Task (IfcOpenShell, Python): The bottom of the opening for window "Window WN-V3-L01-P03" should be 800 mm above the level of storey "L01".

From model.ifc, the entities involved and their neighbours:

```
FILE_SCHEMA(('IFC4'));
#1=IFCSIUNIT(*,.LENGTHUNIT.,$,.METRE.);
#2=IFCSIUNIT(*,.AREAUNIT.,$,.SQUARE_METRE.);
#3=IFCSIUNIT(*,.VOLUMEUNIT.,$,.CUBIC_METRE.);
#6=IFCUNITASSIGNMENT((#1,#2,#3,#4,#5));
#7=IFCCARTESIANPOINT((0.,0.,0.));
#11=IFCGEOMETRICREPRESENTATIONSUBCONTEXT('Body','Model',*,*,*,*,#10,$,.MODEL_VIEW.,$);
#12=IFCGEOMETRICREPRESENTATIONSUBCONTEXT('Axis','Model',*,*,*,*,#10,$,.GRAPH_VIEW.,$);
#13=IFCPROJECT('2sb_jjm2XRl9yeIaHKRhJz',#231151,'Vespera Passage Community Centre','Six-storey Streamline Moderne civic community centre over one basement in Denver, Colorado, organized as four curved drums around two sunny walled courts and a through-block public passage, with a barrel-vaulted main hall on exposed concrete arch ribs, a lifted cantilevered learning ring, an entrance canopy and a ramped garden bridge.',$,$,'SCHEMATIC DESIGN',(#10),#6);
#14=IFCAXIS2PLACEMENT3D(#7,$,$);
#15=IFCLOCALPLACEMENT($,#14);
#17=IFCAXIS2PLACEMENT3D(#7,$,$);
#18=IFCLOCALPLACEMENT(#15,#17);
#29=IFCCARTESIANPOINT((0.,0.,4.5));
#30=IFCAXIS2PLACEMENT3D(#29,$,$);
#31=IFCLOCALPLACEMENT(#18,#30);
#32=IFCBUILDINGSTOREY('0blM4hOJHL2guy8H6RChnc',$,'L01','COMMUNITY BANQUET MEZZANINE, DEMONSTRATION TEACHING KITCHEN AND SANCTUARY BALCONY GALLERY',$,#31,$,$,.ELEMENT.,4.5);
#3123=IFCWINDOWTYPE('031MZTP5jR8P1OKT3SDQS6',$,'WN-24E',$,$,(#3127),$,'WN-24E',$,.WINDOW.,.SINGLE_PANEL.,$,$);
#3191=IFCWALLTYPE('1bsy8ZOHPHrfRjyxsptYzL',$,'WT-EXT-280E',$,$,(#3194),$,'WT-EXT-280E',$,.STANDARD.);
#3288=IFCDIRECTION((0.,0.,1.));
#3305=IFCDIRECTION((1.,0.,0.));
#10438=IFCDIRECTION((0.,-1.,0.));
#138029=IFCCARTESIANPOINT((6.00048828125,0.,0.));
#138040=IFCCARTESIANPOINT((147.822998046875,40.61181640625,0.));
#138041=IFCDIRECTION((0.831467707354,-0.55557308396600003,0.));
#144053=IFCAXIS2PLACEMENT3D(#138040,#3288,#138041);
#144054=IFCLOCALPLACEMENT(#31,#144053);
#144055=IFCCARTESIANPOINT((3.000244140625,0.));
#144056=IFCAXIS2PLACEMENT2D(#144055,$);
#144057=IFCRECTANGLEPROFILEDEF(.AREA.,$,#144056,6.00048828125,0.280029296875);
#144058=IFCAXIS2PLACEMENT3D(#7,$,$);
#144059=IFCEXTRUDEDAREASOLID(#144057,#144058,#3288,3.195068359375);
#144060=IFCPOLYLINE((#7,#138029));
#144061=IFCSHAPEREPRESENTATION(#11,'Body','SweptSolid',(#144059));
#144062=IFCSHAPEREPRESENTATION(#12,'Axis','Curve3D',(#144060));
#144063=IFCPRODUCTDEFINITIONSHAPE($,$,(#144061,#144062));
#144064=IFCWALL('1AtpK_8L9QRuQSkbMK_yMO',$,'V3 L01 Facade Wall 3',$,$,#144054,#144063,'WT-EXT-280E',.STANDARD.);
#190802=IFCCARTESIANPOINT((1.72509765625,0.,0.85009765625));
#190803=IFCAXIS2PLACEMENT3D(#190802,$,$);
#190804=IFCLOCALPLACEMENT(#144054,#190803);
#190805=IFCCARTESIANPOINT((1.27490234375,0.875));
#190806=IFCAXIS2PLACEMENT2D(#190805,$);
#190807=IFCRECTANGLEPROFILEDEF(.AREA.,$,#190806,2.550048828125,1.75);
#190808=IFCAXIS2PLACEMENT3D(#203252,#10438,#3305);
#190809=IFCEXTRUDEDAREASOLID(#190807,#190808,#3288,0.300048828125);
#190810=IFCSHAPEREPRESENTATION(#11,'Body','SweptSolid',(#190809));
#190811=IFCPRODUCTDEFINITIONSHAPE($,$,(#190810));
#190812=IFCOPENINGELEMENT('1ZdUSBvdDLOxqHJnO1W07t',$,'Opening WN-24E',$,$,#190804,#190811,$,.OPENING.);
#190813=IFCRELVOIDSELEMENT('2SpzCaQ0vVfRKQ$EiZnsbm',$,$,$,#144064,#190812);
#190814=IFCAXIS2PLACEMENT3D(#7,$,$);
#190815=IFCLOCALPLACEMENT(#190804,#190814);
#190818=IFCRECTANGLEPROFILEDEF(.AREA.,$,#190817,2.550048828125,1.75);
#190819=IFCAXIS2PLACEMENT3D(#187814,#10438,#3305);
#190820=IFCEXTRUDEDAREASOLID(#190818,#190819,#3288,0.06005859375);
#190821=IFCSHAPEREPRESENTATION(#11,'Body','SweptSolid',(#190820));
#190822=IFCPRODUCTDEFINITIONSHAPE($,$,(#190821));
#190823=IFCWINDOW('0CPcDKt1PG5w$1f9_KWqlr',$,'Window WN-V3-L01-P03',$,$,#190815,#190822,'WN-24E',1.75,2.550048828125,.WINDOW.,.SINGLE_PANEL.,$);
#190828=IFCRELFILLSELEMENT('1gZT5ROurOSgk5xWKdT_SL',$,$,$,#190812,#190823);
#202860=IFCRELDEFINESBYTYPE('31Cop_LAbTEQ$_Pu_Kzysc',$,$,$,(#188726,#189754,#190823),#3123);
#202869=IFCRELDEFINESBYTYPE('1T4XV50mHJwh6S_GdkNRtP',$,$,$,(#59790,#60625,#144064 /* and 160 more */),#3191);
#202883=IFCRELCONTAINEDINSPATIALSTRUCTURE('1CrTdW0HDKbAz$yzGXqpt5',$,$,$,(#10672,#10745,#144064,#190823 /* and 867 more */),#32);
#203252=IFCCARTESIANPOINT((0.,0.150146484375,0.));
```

```python
import numpy as np
import ifcopenshell
import ifcopenshell.api.geometry
import ifcopenshell.geom
import ifcopenshell.util.element
import ifcopenshell.util.placement
import ifcopenshell.util.shape
import ifcopenshell.util.unit

model = ifcopenshell.open("model.ifc")
unit_scale = ifcopenshell.util.unit.calculate_unit_scale(model)

window = model.by_guid("0CPcDKt1PG5w$1f9_KWqlr")
opening = window.FillsVoids[0].RelatingOpeningElement
storey = ifcopenshell.util.element.get_container(window, ifc_class="IfcBuildingStorey")
level = ifcopenshell.util.placement.get_local_placement(storey.ObjectPlacement)[2, 3]

# The opening's origin need not be at the sill, so measure its lowest point.
shape = ifcopenshell.geom.create_shape(ifcopenshell.geom.settings(), opening)
bottom = ifcopenshell.util.shape.get_shape_bottom_elevation(shape, shape.geometry) / unit_scale
dz = level + 0.8 / unit_scale - bottom

shift = np.array([0.0, 0.0, dz])
# The window is placed relative to its opening, so it follows when the opening moves.
matrix = ifcopenshell.util.placement.get_local_placement(opening.ObjectPlacement)
matrix[:3, 3] += shift
ifcopenshell.api.geometry.edit_object_placement(
    model, product=opening, matrix=matrix, is_si=False, should_transform_children=True
)

print(f"moved by {dz * unit_scale:+.3f} m")

model.write("model_v2.ifc")
```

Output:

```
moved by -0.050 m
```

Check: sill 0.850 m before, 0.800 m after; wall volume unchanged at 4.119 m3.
